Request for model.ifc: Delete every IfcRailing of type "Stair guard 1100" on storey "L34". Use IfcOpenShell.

First a look at what the model holds.

```python
import ifcopenshell
import ifcopenshell.util.element

model = ifcopenshell.open("model.ifc")
print(model.schema)
storey = next(s for s in model.by_type("IfcBuildingStorey") if s.Name == "L34")
railings = [e for e in ifcopenshell.util.element.get_decomposition(storey) if e.is_a("IfcRailing")]
seen = {}
for e in railings:
    element_type = ifcopenshell.util.element.get_type(e)
    name = element_type.Name if element_type not in (None, e) else None
    seen[name] = seen.get(name, 0) + 1
for name, count in sorted(seen.items(), key=str):
    print(count, "x", name)
```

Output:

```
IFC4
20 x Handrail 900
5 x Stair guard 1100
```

```python
import ifcopenshell
import ifcopenshell.api.root
import ifcopenshell.util.element

model = ifcopenshell.open("model.ifc")

storey = next(s for s in model.by_type("IfcBuildingStorey") if s.Name == "L34")
railings = [e for e in ifcopenshell.util.element.get_decomposition(storey) if e.is_a("IfcRailing")]
targets = [e for e in railings if (t := ifcopenshell.util.element.get_type(e)) not in (None, e) and t.Name == "Stair guard 1100"]

for e in targets:
    ifcopenshell.api.root.remove_product(model, product=e)
print(len(targets), "removed")

model.write("model_updated.ifc")
```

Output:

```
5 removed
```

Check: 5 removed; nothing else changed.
